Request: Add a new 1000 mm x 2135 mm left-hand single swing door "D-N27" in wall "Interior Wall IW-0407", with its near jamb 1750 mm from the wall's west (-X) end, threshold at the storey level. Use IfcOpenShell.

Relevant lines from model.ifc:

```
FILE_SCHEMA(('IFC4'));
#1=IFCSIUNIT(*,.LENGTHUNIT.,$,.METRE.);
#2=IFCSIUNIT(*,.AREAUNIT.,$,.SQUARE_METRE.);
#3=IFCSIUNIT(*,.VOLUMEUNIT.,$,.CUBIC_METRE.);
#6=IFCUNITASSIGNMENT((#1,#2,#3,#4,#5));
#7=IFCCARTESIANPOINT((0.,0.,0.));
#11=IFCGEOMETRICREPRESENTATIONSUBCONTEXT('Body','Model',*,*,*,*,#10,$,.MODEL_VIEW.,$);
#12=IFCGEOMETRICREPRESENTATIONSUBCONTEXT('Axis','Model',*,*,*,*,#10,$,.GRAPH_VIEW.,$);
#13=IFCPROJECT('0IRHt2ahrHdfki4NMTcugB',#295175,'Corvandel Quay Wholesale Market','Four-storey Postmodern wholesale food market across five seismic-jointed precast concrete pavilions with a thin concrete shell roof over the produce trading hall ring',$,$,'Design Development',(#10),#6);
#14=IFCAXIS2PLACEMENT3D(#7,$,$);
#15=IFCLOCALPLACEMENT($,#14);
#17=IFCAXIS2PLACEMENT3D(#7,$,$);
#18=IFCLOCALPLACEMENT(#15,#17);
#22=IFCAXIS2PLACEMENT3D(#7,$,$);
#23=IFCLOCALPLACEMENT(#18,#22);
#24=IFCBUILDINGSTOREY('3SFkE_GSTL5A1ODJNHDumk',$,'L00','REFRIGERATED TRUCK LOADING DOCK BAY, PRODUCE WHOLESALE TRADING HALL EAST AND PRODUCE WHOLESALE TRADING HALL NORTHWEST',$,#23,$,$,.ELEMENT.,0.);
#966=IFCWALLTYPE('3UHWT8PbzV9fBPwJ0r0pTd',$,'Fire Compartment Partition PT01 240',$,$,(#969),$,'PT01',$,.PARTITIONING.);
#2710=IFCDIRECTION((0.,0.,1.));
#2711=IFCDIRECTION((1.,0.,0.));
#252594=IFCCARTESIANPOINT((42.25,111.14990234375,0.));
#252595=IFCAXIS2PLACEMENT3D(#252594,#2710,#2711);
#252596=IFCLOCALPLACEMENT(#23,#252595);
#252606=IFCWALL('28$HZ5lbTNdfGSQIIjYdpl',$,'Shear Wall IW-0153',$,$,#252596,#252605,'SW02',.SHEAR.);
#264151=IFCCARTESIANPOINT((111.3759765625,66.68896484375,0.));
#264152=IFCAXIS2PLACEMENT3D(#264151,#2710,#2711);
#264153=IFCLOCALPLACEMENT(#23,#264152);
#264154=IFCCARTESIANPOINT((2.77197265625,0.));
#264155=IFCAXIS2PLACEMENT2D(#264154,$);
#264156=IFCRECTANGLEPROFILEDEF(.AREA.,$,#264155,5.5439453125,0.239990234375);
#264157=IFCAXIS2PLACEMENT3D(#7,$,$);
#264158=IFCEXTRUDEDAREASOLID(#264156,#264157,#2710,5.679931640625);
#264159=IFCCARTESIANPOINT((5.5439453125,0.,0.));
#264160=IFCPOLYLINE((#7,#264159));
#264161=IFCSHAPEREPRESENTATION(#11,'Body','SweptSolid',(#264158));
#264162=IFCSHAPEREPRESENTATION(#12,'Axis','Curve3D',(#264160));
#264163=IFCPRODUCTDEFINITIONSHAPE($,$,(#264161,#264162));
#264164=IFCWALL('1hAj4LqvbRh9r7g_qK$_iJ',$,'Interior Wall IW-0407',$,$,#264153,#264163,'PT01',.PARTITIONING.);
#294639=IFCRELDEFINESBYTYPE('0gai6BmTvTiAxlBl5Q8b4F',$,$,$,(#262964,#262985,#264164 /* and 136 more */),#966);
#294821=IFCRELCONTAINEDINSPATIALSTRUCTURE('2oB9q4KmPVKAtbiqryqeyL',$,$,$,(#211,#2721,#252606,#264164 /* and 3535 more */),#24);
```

```python
import numpy as np
import ifcopenshell
import ifcopenshell.api.feature
import ifcopenshell.api.geometry
import ifcopenshell.api.root
import ifcopenshell.api.spatial
import ifcopenshell.geom
import ifcopenshell.util.element
import ifcopenshell.util.placement
import ifcopenshell.util.representation
import ifcopenshell.util.shape
import ifcopenshell.util.unit

model = ifcopenshell.open("model.ifc")
unit_scale = ifcopenshell.util.unit.calculate_unit_scale(model)
settings = ifcopenshell.geom.settings()


def volume(element):
    """Net volume in cubic metres, openings subtracted."""
    shape = ifcopenshell.geom.create_shape(settings, element)
    return ifcopenshell.util.shape.get_volume(shape.geometry)


wall = model.by_guid("1hAj4LqvbRh9r7g_qK$_iJ")
storey = ifcopenshell.util.element.get_container(wall, ifc_class="IfcBuildingStorey")
context = ifcopenshell.util.representation.get_context(model, "Model", "Body", "MODEL_VIEW")
before = volume(wall)

width, height, from_end, sill = 1, 2.135, 1.75, 0.0  # metres

# The wall runs along its own X axis, and the end named is its -X end.
wall_shape = ifcopenshell.geom.create_shape(settings, wall)
x, y, z = ifcopenshell.util.shape.get_vertices(wall_shape.geometry).T
start = x.min() + from_end
face, thickness = float(y.min()), float(y.max() - y.min())
wall_matrix = ifcopenshell.util.placement.get_local_placement(wall.ObjectPlacement)
level = ifcopenshell.util.placement.get_local_placement(storey.ObjectPlacement)[2, 3]


def in_wall(x, y):
    """Placement at x, y metres in the wall's axes, at sill height."""
    matrix = wall_matrix.copy()
    matrix[:, 3] = wall_matrix @ np.array([x / unit_scale, y / unit_scale, 0.0, 1.0])
    matrix[2, 3] = level + sill / unit_scale
    return matrix


# Opening: a box that overshoots both wall faces by 50 mm.
opening = ifcopenshell.api.root.create_entity(model, ifc_class="IfcOpeningElement", predefined_type="OPENING")
box = ifcopenshell.api.geometry.add_wall_representation(
    model, context=context, length=width, height=height, thickness=thickness + 0.1
)
ifcopenshell.api.geometry.assign_representation(model, product=opening, representation=box)
ifcopenshell.api.geometry.edit_object_placement(model, product=opening, matrix=in_wall(start, face - 0.05), is_si=False)
ifcopenshell.api.feature.add_feature(model, feature=opening, element=wall)

door = ifcopenshell.api.root.create_entity(model, ifc_class="IfcDoor", name="D-N27", predefined_type="DOOR")
door.OverallWidth, door.OverallHeight = width / unit_scale, height / unit_scale
door.OperationType = "SINGLE_SWING_LEFT"
body = ifcopenshell.api.geometry.add_door_representation(
    model,
    context=context,
    overall_width=door.OverallWidth,
    overall_height=door.OverallHeight,
    operation_type="SINGLE_SWING_LEFT",
    lining_properties={"LiningDepth": thickness / unit_scale, "ThresholdDepth": thickness / unit_scale},
)
ifcopenshell.api.geometry.assign_representation(model, product=door, representation=body)
ifcopenshell.api.spatial.assign_container(model, products=[door], relating_structure=storey)
ifcopenshell.api.feature.add_filling(model, opening=opening, element=door)

# The lining spans the wall, so the door starts at the wall face.
ifcopenshell.api.geometry.edit_object_placement(model, product=door, matrix=in_wall(start, face), is_si=False)

after = volume(wall)

print(f"wall volume {before:.3f} -> {after:.3f} m3")

model.write("model_edited.ifc")
```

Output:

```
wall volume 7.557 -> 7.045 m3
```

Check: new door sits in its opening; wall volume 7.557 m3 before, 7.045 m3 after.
